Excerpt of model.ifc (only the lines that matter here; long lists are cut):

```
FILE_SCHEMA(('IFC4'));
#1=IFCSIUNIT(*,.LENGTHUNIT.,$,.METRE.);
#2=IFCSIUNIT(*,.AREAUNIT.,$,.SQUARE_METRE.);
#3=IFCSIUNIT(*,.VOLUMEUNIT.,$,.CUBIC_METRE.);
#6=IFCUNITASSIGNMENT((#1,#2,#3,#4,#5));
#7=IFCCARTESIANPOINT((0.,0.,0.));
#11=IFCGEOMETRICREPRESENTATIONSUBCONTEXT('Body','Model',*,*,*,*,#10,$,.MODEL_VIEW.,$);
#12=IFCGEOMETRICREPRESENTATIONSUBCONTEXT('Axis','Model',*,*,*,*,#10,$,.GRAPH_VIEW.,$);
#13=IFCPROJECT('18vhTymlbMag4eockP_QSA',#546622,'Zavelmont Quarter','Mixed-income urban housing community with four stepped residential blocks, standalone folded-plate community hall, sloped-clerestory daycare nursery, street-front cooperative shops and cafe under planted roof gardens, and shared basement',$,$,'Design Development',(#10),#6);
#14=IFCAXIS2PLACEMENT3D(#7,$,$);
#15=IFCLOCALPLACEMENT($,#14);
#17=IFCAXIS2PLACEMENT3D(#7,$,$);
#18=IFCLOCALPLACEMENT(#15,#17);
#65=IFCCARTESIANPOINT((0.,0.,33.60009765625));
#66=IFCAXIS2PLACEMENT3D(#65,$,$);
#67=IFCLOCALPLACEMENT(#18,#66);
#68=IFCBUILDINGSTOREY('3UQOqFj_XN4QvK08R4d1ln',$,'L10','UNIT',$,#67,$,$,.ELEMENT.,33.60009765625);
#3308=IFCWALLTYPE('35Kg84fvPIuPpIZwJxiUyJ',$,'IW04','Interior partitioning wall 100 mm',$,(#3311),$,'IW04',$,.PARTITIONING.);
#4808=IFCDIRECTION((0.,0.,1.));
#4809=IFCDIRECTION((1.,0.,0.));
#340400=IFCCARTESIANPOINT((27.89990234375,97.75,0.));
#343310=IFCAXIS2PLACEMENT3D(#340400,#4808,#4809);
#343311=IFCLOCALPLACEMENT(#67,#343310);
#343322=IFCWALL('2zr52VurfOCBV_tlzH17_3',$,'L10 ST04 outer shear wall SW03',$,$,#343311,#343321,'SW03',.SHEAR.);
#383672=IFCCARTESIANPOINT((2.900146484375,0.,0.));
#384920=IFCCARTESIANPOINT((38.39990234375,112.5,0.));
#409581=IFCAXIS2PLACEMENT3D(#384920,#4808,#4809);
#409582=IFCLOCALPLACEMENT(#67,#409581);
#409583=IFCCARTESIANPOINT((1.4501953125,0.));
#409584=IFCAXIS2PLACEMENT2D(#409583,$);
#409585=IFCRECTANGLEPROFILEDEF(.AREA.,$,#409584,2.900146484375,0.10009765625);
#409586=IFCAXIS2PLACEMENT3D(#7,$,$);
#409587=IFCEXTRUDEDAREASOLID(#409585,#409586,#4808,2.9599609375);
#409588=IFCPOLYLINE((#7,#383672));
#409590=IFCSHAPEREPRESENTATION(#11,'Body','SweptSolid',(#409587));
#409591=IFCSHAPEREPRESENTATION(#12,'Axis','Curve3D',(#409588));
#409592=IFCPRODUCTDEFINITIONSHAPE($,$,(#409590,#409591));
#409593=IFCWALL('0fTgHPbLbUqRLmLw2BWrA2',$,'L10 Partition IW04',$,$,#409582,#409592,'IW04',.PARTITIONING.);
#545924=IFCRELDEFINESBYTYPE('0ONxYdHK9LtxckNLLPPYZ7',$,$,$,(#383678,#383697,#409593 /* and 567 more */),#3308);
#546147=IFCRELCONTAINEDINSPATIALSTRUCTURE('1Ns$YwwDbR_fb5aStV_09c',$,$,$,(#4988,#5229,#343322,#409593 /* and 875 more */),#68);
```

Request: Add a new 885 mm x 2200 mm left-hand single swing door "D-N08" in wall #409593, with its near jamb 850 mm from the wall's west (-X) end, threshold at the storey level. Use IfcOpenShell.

```python
import numpy as np
import ifcopenshell
import ifcopenshell.api.feature
import ifcopenshell.api.geometry
import ifcopenshell.api.root
import ifcopenshell.api.spatial
import ifcopenshell.geom
import ifcopenshell.util.element
import ifcopenshell.util.placement
import ifcopenshell.util.representation
import ifcopenshell.util.shape
import ifcopenshell.util.unit

model = ifcopenshell.open("model.ifc")
unit_scale = ifcopenshell.util.unit.calculate_unit_scale(model)
settings = ifcopenshell.geom.settings()


def volume(element):
    """Net volume in cubic metres, openings subtracted."""
    shape = ifcopenshell.geom.create_shape(settings, element)
    return ifcopenshell.util.shape.get_volume(shape.geometry)


wall = model.by_id(409593)
storey = ifcopenshell.util.element.get_container(wall, ifc_class="IfcBuildingStorey")
context = ifcopenshell.util.representation.get_context(model, "Model", "Body", "MODEL_VIEW")
before = volume(wall)

width, height, from_end, sill = 0.885, 2.2, 0.85, 0.0  # metres

# The wall runs along its own X axis, and the end named is its -X end.
wall_shape = ifcopenshell.geom.create_shape(settings, wall)
x, y, z = ifcopenshell.util.shape.get_vertices(wall_shape.geometry).T
start = x.min() + from_end
face, thickness = float(y.min()), float(y.max() - y.min())
wall_matrix = ifcopenshell.util.placement.get_local_placement(wall.ObjectPlacement)
level = ifcopenshell.util.placement.get_local_placement(storey.ObjectPlacement)[2, 3]


def in_wall(x, y):
    """Placement at x, y metres in the wall's axes, at sill height."""
    matrix = wall_matrix.copy()
    matrix[:, 3] = wall_matrix @ np.array([x / unit_scale, y / unit_scale, 0.0, 1.0])
    matrix[2, 3] = level + sill / unit_scale
    return matrix


# Opening: a box that overshoots both wall faces by 50 mm.
opening = ifcopenshell.api.root.create_entity(model, ifc_class="IfcOpeningElement", predefined_type="OPENING")
box = ifcopenshell.api.geometry.add_wall_representation(
    model, context=context, length=width, height=height, thickness=thickness + 0.1
)
ifcopenshell.api.geometry.assign_representation(model, product=opening, representation=box)
ifcopenshell.api.geometry.edit_object_placement(model, product=opening, matrix=in_wall(start, face - 0.05), is_si=False)
ifcopenshell.api.feature.add_feature(model, feature=opening, element=wall)

door = ifcopenshell.api.root.create_entity(model, ifc_class="IfcDoor", name="D-N08", predefined_type="DOOR")
door.OverallWidth, door.OverallHeight = width / unit_scale, height / unit_scale
door.OperationType = "SINGLE_SWING_LEFT"
body = ifcopenshell.api.geometry.add_door_representation(
    model,
    context=context,
    overall_width=door.OverallWidth,
    overall_height=door.OverallHeight,
    operation_type="SINGLE_SWING_LEFT",
    lining_properties={"LiningDepth": thickness / unit_scale, "ThresholdDepth": thickness / unit_scale},
)
ifcopenshell.api.geometry.assign_representation(model, product=door, representation=body)
ifcopenshell.api.spatial.assign_container(model, products=[door], relating_structure=storey)
ifcopenshell.api.feature.add_filling(model, opening=opening, element=door)

# The lining spans the wall, so the door starts at the wall face.
ifcopenshell.api.geometry.edit_object_placement(model, product=door, matrix=in_wall(start, face), is_si=False)

after = volume(wall)

print(f"wall volume {before:.3f} -> {after:.3f} m3")

model.write("model_rev.ifc")
```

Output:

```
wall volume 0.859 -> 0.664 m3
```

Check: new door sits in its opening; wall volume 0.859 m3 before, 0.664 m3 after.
